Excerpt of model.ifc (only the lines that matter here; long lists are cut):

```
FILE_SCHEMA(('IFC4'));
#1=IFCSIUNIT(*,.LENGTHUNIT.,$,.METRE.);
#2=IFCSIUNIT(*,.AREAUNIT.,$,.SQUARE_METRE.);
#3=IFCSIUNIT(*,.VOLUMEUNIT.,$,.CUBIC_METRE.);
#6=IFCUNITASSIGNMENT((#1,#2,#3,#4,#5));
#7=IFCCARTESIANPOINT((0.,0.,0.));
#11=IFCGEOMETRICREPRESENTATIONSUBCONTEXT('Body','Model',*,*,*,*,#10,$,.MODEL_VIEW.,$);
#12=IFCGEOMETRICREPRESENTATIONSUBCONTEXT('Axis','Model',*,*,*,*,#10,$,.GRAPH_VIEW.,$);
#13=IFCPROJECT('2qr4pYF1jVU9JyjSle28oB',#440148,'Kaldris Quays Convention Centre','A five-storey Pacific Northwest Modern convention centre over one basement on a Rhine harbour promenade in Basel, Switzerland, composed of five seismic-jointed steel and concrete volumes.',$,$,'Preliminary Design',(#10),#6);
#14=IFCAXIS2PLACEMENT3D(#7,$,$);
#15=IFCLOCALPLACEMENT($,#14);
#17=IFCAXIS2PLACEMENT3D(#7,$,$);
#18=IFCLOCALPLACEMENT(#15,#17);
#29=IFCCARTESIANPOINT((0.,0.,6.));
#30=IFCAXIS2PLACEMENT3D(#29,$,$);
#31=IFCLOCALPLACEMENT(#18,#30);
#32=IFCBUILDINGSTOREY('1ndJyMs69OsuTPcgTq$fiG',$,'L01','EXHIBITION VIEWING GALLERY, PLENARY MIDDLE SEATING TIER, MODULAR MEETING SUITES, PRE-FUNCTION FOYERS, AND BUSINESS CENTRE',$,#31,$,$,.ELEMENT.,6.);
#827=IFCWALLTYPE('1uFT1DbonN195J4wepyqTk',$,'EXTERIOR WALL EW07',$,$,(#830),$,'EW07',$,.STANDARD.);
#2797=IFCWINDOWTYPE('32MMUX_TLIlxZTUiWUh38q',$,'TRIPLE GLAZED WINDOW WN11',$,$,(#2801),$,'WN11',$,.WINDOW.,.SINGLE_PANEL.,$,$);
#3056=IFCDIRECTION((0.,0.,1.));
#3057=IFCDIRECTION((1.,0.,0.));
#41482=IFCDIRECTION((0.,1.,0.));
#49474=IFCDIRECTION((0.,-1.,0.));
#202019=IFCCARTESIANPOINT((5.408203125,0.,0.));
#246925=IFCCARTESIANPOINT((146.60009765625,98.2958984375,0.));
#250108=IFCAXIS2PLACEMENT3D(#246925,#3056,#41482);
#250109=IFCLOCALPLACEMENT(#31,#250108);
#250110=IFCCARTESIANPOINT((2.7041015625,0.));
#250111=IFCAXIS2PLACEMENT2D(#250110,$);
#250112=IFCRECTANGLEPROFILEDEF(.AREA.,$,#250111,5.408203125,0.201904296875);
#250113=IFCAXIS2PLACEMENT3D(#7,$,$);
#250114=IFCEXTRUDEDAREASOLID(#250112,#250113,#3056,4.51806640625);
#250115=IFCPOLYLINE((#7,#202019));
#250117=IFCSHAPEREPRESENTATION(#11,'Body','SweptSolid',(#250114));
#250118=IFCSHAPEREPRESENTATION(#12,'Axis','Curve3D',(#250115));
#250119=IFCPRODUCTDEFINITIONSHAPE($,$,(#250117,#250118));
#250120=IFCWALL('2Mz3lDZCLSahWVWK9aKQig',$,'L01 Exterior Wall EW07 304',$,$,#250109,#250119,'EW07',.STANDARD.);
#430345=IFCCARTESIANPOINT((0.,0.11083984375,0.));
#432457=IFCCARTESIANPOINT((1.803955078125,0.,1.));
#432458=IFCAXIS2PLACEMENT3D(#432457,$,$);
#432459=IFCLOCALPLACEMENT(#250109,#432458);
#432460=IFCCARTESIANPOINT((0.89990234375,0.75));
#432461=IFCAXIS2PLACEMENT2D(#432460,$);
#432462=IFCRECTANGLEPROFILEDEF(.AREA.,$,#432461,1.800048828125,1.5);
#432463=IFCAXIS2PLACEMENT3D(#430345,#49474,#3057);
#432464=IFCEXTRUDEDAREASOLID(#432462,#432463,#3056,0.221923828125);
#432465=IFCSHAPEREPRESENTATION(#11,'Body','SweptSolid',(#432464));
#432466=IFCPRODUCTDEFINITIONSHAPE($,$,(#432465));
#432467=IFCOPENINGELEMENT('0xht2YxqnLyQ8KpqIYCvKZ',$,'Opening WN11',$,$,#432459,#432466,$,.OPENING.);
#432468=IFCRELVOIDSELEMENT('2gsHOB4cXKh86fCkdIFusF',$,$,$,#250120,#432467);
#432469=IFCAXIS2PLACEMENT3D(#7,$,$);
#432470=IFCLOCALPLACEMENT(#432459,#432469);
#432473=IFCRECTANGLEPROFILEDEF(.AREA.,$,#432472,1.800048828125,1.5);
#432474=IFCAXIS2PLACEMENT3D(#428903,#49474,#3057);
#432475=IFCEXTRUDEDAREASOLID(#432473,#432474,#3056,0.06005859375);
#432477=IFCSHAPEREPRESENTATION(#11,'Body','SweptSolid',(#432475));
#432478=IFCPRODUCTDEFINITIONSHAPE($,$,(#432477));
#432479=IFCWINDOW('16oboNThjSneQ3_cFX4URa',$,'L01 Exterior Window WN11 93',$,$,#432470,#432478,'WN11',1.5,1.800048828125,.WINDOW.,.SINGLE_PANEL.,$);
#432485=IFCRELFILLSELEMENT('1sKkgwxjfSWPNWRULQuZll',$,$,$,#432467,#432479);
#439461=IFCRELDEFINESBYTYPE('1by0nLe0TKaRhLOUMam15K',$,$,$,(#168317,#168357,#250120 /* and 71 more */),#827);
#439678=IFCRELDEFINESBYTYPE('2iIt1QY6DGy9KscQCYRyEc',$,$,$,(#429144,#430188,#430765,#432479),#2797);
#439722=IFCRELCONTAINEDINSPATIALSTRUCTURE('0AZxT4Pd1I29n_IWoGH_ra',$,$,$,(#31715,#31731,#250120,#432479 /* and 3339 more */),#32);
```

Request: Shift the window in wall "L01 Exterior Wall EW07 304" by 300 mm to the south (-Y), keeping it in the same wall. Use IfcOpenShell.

```python
import ifcopenshell
import ifcopenshell.api.geometry
import ifcopenshell.util.placement
import ifcopenshell.util.unit

model = ifcopenshell.open("model.ifc")
unit_scale = ifcopenshell.util.unit.calculate_unit_scale(model)

window = model.by_guid("16oboNThjSneQ3_cFX4URa")
opening = window.FillsVoids[0].RelatingOpeningElement
wall = opening.VoidsElements[0].RelatingBuildingElement

wall_matrix = ifcopenshell.util.placement.get_local_placement(wall.ObjectPlacement)
shift = wall_matrix[:3, 0] * -0.3 / unit_scale
before = ifcopenshell.util.placement.get_local_placement(window.ObjectPlacement)[:3, 3].copy()

# The window is placed relative to its opening, so it follows when the opening moves.
matrix = ifcopenshell.util.placement.get_local_placement(opening.ObjectPlacement)
matrix[:3, 3] += shift
ifcopenshell.api.geometry.edit_object_placement(
    model, product=opening, matrix=matrix, is_si=False, should_transform_children=True
)

after = ifcopenshell.util.placement.get_local_placement(window.ObjectPlacement)[:3, 3]
print("window moved by", (after - before).round(3) + 0.0)

model.write("model_updated.ifc")
```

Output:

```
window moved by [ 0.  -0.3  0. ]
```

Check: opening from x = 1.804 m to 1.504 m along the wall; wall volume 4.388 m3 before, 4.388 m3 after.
